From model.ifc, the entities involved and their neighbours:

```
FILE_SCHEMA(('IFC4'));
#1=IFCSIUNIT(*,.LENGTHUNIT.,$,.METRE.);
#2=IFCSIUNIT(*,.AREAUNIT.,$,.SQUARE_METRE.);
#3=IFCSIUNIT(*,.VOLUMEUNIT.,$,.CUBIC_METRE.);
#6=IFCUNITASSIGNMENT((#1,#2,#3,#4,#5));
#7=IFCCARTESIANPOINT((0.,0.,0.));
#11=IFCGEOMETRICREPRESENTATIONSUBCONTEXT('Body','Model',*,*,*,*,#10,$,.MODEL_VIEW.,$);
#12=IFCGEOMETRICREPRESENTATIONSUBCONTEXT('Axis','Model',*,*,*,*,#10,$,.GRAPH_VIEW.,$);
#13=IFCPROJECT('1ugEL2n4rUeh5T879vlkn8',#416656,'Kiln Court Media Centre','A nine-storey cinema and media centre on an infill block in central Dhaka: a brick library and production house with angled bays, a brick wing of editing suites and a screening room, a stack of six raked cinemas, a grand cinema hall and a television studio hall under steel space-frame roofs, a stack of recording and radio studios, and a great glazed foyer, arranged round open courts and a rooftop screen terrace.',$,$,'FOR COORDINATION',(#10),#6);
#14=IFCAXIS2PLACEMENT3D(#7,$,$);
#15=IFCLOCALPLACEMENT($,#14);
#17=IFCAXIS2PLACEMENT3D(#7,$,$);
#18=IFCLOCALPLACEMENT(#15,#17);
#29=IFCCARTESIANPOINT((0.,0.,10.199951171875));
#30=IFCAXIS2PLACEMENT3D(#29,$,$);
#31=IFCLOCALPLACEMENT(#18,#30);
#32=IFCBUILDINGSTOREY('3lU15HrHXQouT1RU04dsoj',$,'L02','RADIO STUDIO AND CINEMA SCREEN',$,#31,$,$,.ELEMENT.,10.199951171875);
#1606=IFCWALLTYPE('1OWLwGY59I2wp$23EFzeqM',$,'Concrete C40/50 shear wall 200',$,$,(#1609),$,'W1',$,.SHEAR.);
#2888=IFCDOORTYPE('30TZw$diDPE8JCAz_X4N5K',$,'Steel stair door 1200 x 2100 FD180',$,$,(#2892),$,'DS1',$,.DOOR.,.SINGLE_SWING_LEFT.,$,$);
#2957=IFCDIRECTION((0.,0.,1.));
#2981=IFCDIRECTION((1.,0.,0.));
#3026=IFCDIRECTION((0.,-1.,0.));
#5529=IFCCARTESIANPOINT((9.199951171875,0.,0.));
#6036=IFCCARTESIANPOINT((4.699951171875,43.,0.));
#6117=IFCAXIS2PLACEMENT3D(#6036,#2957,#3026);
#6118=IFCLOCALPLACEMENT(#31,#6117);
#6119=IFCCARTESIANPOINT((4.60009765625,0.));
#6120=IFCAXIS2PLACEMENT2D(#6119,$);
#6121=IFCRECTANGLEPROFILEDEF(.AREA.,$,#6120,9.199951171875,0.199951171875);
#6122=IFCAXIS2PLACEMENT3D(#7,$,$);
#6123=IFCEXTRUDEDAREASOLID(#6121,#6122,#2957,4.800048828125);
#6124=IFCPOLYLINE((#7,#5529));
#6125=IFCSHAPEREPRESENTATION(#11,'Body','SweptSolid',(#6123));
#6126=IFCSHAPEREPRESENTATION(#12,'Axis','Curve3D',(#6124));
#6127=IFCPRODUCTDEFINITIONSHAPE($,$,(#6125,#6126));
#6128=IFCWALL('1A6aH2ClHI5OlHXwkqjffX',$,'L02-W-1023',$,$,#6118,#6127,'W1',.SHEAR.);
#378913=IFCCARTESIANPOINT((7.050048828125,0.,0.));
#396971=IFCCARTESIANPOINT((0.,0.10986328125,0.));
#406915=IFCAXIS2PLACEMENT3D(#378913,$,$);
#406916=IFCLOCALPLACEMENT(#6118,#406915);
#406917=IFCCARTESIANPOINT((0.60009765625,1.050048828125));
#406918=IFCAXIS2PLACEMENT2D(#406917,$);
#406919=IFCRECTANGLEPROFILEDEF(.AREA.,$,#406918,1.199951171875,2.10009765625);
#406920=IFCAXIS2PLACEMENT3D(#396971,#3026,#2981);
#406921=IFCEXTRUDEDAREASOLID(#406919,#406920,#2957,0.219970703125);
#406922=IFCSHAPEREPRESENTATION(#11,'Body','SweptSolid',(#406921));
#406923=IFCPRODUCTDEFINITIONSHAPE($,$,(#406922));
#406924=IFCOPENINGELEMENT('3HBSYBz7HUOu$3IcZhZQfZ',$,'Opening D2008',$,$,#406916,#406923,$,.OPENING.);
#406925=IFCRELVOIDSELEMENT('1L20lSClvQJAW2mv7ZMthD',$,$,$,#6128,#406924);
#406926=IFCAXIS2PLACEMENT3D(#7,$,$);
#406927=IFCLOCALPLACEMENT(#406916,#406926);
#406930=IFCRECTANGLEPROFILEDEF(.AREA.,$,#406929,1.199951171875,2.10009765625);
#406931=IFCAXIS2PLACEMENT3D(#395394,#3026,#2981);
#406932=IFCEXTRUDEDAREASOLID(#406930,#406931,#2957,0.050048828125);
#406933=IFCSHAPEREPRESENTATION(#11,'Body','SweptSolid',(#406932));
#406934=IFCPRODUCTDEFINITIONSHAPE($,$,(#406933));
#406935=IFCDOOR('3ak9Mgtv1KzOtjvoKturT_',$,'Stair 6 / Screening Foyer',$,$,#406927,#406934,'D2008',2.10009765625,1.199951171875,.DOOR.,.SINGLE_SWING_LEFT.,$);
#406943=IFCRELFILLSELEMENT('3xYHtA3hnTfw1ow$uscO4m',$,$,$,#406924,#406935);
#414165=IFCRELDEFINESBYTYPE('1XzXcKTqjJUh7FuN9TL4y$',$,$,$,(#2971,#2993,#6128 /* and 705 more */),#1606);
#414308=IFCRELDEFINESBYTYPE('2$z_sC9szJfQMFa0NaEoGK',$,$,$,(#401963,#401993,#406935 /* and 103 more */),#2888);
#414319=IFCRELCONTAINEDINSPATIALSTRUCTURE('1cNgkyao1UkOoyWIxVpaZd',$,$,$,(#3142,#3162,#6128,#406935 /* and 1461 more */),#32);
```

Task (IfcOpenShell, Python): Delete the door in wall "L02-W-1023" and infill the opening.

```python
import ifcopenshell
import ifcopenshell.api.feature
import ifcopenshell.api.root
import ifcopenshell.geom
import ifcopenshell.util.shape

model = ifcopenshell.open("model.ifc")
settings = ifcopenshell.geom.settings()


def volume(element):
    """Net volume in cubic metres, openings subtracted."""
    shape = ifcopenshell.geom.create_shape(settings, element)
    return ifcopenshell.util.shape.get_volume(shape.geometry)


door = model.by_guid("3ak9Mgtv1KzOtjvoKturT_")
opening = door.FillsVoids[0].RelatingOpeningElement
wall = opening.VoidsElements[0].RelatingBuildingElement
before = volume(wall)

ifcopenshell.api.root.remove_product(model, product=door)
ifcopenshell.api.feature.remove_feature(model, feature=opening)

after = volume(wall)

print(f"wall volume {before:.3f} -> {after:.3f} m3")

model.write("model_rev.ifc")
```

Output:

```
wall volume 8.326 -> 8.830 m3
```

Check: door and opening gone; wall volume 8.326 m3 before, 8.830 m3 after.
